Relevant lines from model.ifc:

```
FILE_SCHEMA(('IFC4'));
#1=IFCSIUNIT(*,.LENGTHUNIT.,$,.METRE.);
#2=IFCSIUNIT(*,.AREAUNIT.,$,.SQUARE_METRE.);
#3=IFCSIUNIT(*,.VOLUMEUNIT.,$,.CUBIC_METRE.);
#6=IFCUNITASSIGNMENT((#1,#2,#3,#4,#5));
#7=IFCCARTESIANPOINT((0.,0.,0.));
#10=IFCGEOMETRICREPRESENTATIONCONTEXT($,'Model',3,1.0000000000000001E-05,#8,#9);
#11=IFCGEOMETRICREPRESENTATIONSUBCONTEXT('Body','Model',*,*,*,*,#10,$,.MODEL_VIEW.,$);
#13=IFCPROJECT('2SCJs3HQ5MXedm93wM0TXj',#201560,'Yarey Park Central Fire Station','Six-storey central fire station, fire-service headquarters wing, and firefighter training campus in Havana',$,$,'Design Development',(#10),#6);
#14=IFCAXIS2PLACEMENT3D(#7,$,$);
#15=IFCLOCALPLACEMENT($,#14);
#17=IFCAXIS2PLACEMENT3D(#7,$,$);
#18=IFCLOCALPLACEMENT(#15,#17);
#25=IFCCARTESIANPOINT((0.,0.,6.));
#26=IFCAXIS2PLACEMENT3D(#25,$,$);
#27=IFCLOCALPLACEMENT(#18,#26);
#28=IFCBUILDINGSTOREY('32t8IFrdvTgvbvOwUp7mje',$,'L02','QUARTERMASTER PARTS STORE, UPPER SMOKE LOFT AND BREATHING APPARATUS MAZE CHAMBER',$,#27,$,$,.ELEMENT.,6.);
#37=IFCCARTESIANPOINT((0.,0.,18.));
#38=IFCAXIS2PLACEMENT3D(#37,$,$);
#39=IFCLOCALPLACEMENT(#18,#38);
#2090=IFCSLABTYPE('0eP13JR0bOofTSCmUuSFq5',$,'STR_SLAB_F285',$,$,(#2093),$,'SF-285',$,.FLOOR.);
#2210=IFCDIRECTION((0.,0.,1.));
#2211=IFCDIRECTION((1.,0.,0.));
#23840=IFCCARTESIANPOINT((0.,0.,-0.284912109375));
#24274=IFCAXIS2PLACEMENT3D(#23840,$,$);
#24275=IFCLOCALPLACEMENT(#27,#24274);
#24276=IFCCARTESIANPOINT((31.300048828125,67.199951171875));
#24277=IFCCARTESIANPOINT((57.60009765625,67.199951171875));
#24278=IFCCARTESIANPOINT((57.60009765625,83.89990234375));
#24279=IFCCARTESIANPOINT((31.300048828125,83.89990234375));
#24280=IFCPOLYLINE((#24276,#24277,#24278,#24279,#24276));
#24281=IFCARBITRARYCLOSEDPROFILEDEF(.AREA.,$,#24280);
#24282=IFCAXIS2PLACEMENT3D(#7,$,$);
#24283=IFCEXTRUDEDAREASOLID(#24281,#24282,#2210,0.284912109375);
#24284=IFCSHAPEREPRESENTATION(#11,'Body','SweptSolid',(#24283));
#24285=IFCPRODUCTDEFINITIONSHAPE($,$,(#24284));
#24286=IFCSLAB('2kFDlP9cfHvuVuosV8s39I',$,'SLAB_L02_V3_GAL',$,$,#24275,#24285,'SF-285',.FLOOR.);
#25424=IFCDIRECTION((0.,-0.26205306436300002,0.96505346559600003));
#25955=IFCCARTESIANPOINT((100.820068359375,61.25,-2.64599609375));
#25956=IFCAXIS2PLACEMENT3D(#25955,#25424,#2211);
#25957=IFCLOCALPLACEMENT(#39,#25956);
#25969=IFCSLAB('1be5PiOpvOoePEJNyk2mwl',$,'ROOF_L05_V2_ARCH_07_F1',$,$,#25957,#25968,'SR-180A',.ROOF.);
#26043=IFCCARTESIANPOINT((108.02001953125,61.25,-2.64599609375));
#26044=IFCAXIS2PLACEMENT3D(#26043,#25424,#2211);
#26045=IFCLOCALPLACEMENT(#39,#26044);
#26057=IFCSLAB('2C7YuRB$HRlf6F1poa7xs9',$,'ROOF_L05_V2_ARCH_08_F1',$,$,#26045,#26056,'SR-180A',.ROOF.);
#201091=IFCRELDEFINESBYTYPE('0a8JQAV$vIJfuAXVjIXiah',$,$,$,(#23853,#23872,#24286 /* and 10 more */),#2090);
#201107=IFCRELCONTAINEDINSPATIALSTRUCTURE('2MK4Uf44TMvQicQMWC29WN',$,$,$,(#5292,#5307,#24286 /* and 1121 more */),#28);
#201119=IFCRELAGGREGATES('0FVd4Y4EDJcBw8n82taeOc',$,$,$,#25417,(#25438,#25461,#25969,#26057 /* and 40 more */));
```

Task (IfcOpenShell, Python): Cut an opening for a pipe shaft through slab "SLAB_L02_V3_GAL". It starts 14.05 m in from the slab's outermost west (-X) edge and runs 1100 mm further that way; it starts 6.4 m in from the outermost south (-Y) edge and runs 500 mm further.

```python
import numpy as np
import ifcopenshell
import ifcopenshell.api.feature
import ifcopenshell.api.geometry
import ifcopenshell.api.root
import ifcopenshell.geom
import ifcopenshell.util.placement
import ifcopenshell.util.representation
import ifcopenshell.util.shape
import ifcopenshell.util.unit

model = ifcopenshell.open("model.ifc")
unit_scale = ifcopenshell.util.unit.calculate_unit_scale(model)
settings = ifcopenshell.geom.settings()


def volume(element):
    """Net volume in cubic metres, openings subtracted."""
    shape = ifcopenshell.geom.create_shape(settings, element)
    return ifcopenshell.util.shape.get_volume(shape.geometry)


slab = model.by_id(24286)
before = volume(slab)

# Extent in the slab's own axes, in metres. The edges named are its -X and -Y sides.
slab_shape = ifcopenshell.geom.create_shape(settings, slab)
vertices = ifcopenshell.util.shape.get_vertices(slab_shape.geometry)
x_min, y_min, bottom = vertices.min(axis=0)
top = vertices[:, 2].max()

opening = ifcopenshell.api.root.create_entity(model, ifc_class="IfcOpeningElement", name="Pipe shaft opening", predefined_type="OPENING")
context = ifcopenshell.util.representation.get_context(model, "Model", "Body", "MODEL_VIEW")
width, depth = 1.1, 0.5
outline = [(0.0, 0.0), (width, 0.0), (width, depth), (0.0, depth), (0.0, 0.0)]
# Overshoot both faces by 50 mm so the cut is clean.
shape = ifcopenshell.api.geometry.add_slab_representation(
    model, context=context, depth=top - bottom + 0.1, polyline=outline
)
ifcopenshell.api.geometry.assign_representation(model, product=opening, representation=shape)

matrix = ifcopenshell.util.placement.get_local_placement(slab.ObjectPlacement)
matrix[:, 3] = matrix @ np.append(np.array([x_min + 14.05, y_min + 6.4, bottom - 0.05]) / unit_scale, 1.0)
ifcopenshell.api.geometry.edit_object_placement(model, product=opening, matrix=matrix, is_si=False)
ifcopenshell.api.feature.add_feature(model, feature=opening, element=slab)

after = volume(slab)

print(f"slab volume {before:.3f} -> {after:.3f} m3")

model.write("model_v2.ifc")
```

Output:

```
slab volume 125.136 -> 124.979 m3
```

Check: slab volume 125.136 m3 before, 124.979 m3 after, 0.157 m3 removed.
